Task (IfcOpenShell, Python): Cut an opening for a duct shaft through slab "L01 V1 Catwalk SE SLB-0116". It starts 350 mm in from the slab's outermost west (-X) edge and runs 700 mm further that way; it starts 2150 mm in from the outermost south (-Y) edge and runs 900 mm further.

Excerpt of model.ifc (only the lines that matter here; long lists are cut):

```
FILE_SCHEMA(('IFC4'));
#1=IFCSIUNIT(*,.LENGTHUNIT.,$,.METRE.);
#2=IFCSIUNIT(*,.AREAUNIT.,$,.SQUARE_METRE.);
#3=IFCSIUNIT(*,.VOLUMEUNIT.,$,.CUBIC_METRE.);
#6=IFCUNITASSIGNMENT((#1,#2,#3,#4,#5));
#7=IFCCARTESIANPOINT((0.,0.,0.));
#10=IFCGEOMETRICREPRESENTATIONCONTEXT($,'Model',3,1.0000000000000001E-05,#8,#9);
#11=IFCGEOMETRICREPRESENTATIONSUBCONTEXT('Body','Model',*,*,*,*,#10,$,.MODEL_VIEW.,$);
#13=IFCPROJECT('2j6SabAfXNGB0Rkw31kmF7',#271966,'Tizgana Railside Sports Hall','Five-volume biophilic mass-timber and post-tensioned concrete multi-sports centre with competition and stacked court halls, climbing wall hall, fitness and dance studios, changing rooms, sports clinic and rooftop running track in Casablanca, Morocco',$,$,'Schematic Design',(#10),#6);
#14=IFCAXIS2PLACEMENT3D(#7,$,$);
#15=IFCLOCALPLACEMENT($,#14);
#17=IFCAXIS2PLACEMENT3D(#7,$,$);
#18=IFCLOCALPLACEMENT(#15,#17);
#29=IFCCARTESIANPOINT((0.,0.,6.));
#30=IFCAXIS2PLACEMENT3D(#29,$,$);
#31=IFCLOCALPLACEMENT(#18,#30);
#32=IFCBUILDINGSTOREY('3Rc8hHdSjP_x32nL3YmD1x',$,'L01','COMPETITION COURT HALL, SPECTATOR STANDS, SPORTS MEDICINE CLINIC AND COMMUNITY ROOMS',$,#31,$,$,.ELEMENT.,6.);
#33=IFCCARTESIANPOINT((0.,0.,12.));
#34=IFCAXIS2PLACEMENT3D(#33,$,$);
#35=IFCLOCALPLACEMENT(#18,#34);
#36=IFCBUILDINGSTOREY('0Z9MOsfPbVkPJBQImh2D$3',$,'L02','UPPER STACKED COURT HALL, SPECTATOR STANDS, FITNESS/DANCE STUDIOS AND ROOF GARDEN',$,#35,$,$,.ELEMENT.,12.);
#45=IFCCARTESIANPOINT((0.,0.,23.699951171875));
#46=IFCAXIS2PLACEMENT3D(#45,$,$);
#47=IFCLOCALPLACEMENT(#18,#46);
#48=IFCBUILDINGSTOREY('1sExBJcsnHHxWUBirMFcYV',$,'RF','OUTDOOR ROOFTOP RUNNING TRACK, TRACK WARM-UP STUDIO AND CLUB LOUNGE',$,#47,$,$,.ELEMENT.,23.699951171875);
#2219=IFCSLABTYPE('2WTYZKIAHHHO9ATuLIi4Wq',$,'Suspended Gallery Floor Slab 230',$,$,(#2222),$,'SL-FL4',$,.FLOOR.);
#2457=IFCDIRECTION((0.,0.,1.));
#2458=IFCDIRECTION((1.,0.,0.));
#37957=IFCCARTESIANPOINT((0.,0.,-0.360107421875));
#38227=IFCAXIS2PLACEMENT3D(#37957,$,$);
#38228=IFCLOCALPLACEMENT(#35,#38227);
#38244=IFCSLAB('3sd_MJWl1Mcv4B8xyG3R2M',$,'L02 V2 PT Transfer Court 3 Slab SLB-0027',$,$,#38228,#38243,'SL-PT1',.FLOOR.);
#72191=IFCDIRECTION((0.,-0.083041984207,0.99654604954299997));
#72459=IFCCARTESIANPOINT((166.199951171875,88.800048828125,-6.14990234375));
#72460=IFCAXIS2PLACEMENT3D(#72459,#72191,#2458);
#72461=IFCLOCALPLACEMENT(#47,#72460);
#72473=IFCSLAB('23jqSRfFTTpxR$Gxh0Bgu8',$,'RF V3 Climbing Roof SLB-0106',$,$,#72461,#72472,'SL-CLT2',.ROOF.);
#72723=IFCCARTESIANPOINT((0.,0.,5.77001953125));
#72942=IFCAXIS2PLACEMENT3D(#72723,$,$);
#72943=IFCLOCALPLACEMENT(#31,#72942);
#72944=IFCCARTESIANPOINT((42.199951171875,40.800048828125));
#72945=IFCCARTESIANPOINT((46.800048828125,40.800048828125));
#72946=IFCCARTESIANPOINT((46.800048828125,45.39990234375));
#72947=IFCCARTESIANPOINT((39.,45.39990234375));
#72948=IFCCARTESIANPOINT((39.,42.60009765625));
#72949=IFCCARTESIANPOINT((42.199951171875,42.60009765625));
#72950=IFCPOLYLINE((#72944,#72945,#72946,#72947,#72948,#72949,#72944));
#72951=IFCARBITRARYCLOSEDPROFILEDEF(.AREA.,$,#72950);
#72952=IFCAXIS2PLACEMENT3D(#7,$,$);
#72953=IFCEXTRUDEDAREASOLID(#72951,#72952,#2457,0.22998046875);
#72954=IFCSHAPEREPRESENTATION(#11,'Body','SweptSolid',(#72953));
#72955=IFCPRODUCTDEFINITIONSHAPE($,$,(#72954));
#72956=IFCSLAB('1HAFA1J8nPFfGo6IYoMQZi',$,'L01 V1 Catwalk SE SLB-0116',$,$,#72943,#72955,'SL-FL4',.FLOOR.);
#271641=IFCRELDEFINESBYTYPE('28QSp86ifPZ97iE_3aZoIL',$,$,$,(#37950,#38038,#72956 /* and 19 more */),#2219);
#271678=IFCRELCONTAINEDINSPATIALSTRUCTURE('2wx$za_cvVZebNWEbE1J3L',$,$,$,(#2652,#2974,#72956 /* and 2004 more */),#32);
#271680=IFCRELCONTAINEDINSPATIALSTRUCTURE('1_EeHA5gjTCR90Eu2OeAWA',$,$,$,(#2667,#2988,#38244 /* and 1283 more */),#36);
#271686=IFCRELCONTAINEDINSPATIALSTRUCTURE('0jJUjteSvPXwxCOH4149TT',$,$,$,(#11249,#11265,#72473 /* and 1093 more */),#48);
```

```python
import numpy as np
import ifcopenshell
import ifcopenshell.api.feature
import ifcopenshell.api.geometry
import ifcopenshell.api.root
import ifcopenshell.geom
import ifcopenshell.util.placement
import ifcopenshell.util.representation
import ifcopenshell.util.shape
import ifcopenshell.util.unit

model = ifcopenshell.open("model.ifc")
unit_scale = ifcopenshell.util.unit.calculate_unit_scale(model)
settings = ifcopenshell.geom.settings()


def volume(element):
    """Net volume in cubic metres, openings subtracted."""
    shape = ifcopenshell.geom.create_shape(settings, element)
    return ifcopenshell.util.shape.get_volume(shape.geometry)


slab = model.by_id(72956)
before = volume(slab)

# Extent in the slab's own axes, in metres. The edges named are its -X and -Y sides.
slab_shape = ifcopenshell.geom.create_shape(settings, slab)
vertices = ifcopenshell.util.shape.get_vertices(slab_shape.geometry)
x_min, y_min, bottom = vertices.min(axis=0)
top = vertices[:, 2].max()

opening = ifcopenshell.api.root.create_entity(model, ifc_class="IfcOpeningElement", name="Duct shaft opening", predefined_type="OPENING")
context = ifcopenshell.util.representation.get_context(model, "Model", "Body", "MODEL_VIEW")
width, depth = 0.7, 0.9
outline = [(0.0, 0.0), (width, 0.0), (width, depth), (0.0, depth), (0.0, 0.0)]
# Overshoot both faces by 50 mm so the cut is clean.
shape = ifcopenshell.api.geometry.add_slab_representation(
    model, context=context, depth=top - bottom + 0.1, polyline=outline
)
ifcopenshell.api.geometry.assign_representation(model, product=opening, representation=shape)

matrix = ifcopenshell.util.placement.get_local_placement(slab.ObjectPlacement)
matrix[:, 3] = matrix @ np.append(np.array([x_min + 0.35, y_min + 2.15, bottom - 0.05]) / unit_scale, 1.0)
ifcopenshell.api.geometry.edit_object_placement(model, product=opening, matrix=matrix, is_si=False)
ifcopenshell.api.feature.add_feature(model, feature=opening, element=slab)

after = volume(slab)

print(f"slab volume {before:.3f} -> {after:.3f} m3")

model.write("model-out.ifc")
```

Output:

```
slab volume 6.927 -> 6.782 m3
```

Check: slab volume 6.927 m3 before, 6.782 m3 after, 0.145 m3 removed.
